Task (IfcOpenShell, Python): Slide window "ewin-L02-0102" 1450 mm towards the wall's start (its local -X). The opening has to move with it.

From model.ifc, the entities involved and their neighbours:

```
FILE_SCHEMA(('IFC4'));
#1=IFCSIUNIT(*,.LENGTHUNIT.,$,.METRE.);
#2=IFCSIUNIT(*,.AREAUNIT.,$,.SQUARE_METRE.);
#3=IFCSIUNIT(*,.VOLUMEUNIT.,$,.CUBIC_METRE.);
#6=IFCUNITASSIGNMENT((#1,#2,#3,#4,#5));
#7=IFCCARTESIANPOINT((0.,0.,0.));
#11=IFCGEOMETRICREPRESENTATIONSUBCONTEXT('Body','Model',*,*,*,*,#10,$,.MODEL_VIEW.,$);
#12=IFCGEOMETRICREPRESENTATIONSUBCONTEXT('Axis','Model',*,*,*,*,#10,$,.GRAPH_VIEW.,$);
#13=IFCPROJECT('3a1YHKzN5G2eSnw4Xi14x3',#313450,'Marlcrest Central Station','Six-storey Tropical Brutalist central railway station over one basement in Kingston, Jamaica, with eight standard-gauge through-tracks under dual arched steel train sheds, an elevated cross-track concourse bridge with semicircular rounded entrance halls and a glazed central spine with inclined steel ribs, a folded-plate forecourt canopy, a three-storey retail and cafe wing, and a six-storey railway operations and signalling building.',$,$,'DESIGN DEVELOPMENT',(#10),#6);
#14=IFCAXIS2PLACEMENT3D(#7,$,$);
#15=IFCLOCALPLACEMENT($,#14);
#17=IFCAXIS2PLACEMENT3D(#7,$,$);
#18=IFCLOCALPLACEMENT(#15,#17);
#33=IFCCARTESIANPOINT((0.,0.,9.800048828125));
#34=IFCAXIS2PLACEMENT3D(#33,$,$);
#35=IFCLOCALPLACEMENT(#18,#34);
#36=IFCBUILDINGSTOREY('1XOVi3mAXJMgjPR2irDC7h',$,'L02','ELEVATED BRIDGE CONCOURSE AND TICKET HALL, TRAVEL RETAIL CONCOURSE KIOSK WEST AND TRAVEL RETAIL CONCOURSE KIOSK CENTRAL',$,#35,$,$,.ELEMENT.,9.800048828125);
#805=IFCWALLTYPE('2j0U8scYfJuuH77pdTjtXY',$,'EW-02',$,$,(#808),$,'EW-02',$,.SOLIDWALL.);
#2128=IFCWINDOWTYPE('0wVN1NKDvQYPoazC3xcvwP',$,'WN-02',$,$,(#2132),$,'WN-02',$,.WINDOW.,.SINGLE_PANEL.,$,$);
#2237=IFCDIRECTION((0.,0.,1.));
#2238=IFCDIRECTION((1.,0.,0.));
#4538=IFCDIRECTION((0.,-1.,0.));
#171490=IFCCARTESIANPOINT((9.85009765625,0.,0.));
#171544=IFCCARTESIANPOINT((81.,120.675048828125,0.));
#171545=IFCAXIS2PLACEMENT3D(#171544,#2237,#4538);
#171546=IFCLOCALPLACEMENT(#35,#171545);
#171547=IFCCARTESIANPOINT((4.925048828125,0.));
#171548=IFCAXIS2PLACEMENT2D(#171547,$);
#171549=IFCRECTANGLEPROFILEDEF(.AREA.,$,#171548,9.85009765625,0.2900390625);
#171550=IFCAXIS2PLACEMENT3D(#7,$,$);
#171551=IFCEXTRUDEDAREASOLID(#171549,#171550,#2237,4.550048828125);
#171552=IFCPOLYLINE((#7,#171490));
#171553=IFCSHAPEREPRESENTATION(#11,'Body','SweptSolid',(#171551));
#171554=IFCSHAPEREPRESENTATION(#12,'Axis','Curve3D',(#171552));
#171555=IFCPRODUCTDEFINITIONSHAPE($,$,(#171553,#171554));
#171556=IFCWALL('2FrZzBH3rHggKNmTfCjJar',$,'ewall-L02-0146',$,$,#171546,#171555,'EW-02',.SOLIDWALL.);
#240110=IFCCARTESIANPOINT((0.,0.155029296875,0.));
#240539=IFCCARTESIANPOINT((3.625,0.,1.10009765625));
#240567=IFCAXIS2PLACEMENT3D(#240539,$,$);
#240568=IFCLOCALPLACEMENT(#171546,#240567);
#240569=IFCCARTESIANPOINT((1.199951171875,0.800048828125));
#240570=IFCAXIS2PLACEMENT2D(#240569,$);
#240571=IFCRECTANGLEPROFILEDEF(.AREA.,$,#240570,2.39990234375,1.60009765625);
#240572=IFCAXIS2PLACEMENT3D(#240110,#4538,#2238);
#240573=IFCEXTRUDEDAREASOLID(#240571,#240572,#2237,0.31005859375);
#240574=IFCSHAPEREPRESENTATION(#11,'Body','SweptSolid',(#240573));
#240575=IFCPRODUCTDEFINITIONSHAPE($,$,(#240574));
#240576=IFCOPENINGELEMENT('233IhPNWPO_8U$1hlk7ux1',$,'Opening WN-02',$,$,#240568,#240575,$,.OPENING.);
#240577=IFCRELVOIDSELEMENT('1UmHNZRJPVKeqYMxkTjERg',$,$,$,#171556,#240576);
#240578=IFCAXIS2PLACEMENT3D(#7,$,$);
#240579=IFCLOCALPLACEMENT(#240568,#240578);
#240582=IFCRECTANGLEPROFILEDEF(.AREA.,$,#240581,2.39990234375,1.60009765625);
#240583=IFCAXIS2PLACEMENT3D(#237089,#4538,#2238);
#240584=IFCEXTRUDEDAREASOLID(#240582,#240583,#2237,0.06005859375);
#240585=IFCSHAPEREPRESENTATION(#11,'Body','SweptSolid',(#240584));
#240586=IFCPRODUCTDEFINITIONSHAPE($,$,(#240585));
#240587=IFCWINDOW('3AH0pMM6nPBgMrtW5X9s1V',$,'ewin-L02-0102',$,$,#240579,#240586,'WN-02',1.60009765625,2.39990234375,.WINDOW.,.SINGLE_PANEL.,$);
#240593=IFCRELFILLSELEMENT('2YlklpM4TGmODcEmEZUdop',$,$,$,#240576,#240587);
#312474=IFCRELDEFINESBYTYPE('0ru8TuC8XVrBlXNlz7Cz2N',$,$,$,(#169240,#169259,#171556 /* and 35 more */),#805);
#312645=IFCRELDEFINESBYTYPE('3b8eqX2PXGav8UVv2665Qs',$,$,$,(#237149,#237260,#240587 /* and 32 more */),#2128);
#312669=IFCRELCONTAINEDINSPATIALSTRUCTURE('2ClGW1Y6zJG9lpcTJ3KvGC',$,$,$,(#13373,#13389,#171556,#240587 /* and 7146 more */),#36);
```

```python
import ifcopenshell
import ifcopenshell.api.geometry
import ifcopenshell.util.placement

model = ifcopenshell.open("model.ifc")

window = model.by_id(240587)
opening = window.FillsVoids[0].RelatingOpeningElement
wall = opening.VoidsElements[0].RelatingBuildingElement

wall_matrix = ifcopenshell.util.placement.get_local_placement(wall.ObjectPlacement)
shift = wall_matrix[:3, 0] * -1.45
before = ifcopenshell.util.placement.get_local_placement(window.ObjectPlacement)[:3, 3].copy()

# The window is placed relative to its opening, so it follows when the opening moves.
matrix = ifcopenshell.util.placement.get_local_placement(opening.ObjectPlacement)
matrix[:3, 3] += shift
ifcopenshell.api.geometry.edit_object_placement(
    model, product=opening, matrix=matrix, is_si=False, should_transform_children=True
)

after = ifcopenshell.util.placement.get_local_placement(window.ObjectPlacement)[:3, 3]
print("window moved by", (after - before).round(3) + 0.0)

model.write("model_rev.ifc")
```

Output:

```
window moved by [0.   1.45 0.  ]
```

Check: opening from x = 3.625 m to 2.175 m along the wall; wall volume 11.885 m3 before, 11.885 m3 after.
